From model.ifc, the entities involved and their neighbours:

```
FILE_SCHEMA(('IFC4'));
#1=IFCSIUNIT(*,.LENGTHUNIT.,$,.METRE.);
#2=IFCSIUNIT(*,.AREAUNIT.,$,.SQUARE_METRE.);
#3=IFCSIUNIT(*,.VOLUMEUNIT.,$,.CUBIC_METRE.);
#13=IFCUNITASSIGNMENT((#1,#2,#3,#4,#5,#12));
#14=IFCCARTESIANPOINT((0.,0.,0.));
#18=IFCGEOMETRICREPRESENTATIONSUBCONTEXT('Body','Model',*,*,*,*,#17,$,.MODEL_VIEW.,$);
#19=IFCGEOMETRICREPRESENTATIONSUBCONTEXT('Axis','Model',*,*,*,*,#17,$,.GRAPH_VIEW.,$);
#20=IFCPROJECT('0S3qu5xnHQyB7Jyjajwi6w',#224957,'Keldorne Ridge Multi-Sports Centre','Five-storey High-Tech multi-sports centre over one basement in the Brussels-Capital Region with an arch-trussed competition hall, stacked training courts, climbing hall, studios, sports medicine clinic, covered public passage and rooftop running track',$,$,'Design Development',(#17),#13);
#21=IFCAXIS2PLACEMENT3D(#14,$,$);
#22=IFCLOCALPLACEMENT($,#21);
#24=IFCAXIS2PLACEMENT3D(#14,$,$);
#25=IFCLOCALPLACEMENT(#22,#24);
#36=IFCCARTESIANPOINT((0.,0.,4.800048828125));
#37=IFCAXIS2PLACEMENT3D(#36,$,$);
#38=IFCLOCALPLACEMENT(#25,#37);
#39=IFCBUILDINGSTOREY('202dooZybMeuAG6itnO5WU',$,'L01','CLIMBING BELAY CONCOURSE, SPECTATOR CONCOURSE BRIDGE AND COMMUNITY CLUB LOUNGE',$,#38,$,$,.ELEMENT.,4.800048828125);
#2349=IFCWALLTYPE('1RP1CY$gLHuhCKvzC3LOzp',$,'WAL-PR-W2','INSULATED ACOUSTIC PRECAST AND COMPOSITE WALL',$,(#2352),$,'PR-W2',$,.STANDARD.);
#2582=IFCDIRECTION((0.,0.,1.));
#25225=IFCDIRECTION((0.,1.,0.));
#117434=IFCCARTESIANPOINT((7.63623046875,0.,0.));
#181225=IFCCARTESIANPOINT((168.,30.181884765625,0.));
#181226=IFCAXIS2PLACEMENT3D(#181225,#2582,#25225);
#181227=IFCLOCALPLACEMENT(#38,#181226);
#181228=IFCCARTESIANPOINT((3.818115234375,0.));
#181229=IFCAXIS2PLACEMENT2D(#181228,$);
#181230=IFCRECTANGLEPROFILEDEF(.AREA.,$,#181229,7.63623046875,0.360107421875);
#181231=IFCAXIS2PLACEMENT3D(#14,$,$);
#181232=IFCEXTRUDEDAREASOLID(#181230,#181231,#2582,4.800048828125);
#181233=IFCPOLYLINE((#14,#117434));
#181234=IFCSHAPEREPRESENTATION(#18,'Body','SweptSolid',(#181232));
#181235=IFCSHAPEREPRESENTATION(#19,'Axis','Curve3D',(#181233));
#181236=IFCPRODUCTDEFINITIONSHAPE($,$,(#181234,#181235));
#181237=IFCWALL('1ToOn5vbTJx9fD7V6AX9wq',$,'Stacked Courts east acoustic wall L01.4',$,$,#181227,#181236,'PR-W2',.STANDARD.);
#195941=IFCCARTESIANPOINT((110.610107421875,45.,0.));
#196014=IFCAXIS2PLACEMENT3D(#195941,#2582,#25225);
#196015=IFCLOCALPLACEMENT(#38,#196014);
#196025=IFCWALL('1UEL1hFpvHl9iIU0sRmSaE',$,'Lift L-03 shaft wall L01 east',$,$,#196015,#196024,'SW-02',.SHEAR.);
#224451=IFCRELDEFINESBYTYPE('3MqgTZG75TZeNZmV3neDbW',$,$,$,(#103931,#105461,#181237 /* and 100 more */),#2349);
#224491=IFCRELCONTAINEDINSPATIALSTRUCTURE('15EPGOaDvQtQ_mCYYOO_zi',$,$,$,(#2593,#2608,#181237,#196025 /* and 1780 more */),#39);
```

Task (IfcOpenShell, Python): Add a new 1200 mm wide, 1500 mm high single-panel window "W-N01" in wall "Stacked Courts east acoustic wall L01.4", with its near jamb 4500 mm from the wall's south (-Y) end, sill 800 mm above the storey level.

```python
import numpy as np
import ifcopenshell
import ifcopenshell.api.feature
import ifcopenshell.api.geometry
import ifcopenshell.api.root
import ifcopenshell.api.spatial
import ifcopenshell.geom
import ifcopenshell.util.element
import ifcopenshell.util.placement
import ifcopenshell.util.representation
import ifcopenshell.util.shape
import ifcopenshell.util.unit

model = ifcopenshell.open("model.ifc")
unit_scale = ifcopenshell.util.unit.calculate_unit_scale(model)
settings = ifcopenshell.geom.settings()


def volume(element):
    """Net volume in cubic metres, openings subtracted."""
    shape = ifcopenshell.geom.create_shape(settings, element)
    return ifcopenshell.util.shape.get_volume(shape.geometry)


wall = model.by_guid("1ToOn5vbTJx9fD7V6AX9wq")
storey = ifcopenshell.util.element.get_container(wall, ifc_class="IfcBuildingStorey")
context = ifcopenshell.util.representation.get_context(model, "Model", "Body", "MODEL_VIEW")
before = volume(wall)

width, height, from_end, sill = 1.2, 1.5, 4.5, 0.8  # metres

# The wall runs along its own X axis, and the end named is its -X end.
wall_shape = ifcopenshell.geom.create_shape(settings, wall)
x, y, z = ifcopenshell.util.shape.get_vertices(wall_shape.geometry).T
start = x.min() + from_end
face, thickness = float(y.min()), float(y.max() - y.min())
wall_matrix = ifcopenshell.util.placement.get_local_placement(wall.ObjectPlacement)
level = ifcopenshell.util.placement.get_local_placement(storey.ObjectPlacement)[2, 3]


def in_wall(x, y):
    """Placement at x, y metres in the wall's axes, at sill height."""
    matrix = wall_matrix.copy()
    matrix[:, 3] = wall_matrix @ np.array([x / unit_scale, y / unit_scale, 0.0, 1.0])
    matrix[2, 3] = level + sill / unit_scale
    return matrix


# Opening: a box that overshoots both wall faces by 50 mm.
opening = ifcopenshell.api.root.create_entity(model, ifc_class="IfcOpeningElement", predefined_type="OPENING")
box = ifcopenshell.api.geometry.add_wall_representation(
    model, context=context, length=width, height=height, thickness=thickness + 0.1
)
ifcopenshell.api.geometry.assign_representation(model, product=opening, representation=box)
ifcopenshell.api.geometry.edit_object_placement(model, product=opening, matrix=in_wall(start, face - 0.05), is_si=False)
ifcopenshell.api.feature.add_feature(model, feature=opening, element=wall)

window = ifcopenshell.api.root.create_entity(model, ifc_class="IfcWindow", name="W-N01", predefined_type="WINDOW")
window.OverallWidth, window.OverallHeight = width / unit_scale, height / unit_scale
window.PartitioningType = "SINGLE_PANEL"
body = ifcopenshell.api.geometry.add_window_representation(
    model,
    context=context,
    overall_width=window.OverallWidth,
    overall_height=window.OverallHeight,
    partition_type="SINGLE_PANEL",
)
ifcopenshell.api.geometry.assign_representation(model, product=window, representation=body)
ifcopenshell.api.spatial.assign_container(model, products=[window], relating_structure=storey)
ifcopenshell.api.feature.add_filling(model, opening=opening, element=window)

# Centre the window in the wall's thickness.
ifcopenshell.api.geometry.edit_object_placement(model, product=window, matrix=in_wall(start, face), is_si=False)
window_shape = ifcopenshell.geom.create_shape(settings, window)
depth = ifcopenshell.util.shape.get_vertices(window_shape.geometry)[:, 1]
offset = face + thickness / 2 - (depth.min() + depth.max()) / 2
ifcopenshell.api.geometry.edit_object_placement(model, product=window, matrix=in_wall(start, offset), is_si=False)

after = volume(wall)

print(f"wall volume {before:.3f} -> {after:.3f} m3")

model.write("model_edited.ifc")
```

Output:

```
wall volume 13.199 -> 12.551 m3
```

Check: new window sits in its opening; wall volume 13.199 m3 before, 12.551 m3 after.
